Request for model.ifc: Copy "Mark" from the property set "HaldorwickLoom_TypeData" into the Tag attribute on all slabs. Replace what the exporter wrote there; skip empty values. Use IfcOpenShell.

First a look at what the model holds.

```python
import ifcopenshell
import ifcopenshell.util.element

model = ifcopenshell.open("model.ifc")
print(model.schema)
slabs = model.by_type("IfcSlab")
print(len(slabs), "slabs")
for e in slabs[:8]:
    source = ifcopenshell.util.element.get_pset(e, "HaldorwickLoom_TypeData", "Mark")
    target = e.Tag
    print(e.id(), repr(source), repr(target), sep=" | ")
```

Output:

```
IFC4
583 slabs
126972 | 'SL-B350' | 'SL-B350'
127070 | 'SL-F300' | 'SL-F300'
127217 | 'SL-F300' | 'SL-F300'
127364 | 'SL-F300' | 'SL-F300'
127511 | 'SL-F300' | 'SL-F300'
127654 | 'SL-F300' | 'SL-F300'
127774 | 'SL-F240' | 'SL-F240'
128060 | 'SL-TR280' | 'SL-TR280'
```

```python
import ifcopenshell
import ifcopenshell.util.element

model = ifcopenshell.open("model.ifc")

count = 0
for e in model.by_type("IfcSlab"):
    value = ifcopenshell.util.element.get_pset(e, "HaldorwickLoom_TypeData", "Mark")
    current = e.Tag
    if not value or not value.strip() or current == value:
        continue
    e.Tag = value
    count += 1

print(count, "slabs updated")

model.write("model_updated.ifc")
```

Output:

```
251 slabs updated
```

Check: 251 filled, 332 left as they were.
